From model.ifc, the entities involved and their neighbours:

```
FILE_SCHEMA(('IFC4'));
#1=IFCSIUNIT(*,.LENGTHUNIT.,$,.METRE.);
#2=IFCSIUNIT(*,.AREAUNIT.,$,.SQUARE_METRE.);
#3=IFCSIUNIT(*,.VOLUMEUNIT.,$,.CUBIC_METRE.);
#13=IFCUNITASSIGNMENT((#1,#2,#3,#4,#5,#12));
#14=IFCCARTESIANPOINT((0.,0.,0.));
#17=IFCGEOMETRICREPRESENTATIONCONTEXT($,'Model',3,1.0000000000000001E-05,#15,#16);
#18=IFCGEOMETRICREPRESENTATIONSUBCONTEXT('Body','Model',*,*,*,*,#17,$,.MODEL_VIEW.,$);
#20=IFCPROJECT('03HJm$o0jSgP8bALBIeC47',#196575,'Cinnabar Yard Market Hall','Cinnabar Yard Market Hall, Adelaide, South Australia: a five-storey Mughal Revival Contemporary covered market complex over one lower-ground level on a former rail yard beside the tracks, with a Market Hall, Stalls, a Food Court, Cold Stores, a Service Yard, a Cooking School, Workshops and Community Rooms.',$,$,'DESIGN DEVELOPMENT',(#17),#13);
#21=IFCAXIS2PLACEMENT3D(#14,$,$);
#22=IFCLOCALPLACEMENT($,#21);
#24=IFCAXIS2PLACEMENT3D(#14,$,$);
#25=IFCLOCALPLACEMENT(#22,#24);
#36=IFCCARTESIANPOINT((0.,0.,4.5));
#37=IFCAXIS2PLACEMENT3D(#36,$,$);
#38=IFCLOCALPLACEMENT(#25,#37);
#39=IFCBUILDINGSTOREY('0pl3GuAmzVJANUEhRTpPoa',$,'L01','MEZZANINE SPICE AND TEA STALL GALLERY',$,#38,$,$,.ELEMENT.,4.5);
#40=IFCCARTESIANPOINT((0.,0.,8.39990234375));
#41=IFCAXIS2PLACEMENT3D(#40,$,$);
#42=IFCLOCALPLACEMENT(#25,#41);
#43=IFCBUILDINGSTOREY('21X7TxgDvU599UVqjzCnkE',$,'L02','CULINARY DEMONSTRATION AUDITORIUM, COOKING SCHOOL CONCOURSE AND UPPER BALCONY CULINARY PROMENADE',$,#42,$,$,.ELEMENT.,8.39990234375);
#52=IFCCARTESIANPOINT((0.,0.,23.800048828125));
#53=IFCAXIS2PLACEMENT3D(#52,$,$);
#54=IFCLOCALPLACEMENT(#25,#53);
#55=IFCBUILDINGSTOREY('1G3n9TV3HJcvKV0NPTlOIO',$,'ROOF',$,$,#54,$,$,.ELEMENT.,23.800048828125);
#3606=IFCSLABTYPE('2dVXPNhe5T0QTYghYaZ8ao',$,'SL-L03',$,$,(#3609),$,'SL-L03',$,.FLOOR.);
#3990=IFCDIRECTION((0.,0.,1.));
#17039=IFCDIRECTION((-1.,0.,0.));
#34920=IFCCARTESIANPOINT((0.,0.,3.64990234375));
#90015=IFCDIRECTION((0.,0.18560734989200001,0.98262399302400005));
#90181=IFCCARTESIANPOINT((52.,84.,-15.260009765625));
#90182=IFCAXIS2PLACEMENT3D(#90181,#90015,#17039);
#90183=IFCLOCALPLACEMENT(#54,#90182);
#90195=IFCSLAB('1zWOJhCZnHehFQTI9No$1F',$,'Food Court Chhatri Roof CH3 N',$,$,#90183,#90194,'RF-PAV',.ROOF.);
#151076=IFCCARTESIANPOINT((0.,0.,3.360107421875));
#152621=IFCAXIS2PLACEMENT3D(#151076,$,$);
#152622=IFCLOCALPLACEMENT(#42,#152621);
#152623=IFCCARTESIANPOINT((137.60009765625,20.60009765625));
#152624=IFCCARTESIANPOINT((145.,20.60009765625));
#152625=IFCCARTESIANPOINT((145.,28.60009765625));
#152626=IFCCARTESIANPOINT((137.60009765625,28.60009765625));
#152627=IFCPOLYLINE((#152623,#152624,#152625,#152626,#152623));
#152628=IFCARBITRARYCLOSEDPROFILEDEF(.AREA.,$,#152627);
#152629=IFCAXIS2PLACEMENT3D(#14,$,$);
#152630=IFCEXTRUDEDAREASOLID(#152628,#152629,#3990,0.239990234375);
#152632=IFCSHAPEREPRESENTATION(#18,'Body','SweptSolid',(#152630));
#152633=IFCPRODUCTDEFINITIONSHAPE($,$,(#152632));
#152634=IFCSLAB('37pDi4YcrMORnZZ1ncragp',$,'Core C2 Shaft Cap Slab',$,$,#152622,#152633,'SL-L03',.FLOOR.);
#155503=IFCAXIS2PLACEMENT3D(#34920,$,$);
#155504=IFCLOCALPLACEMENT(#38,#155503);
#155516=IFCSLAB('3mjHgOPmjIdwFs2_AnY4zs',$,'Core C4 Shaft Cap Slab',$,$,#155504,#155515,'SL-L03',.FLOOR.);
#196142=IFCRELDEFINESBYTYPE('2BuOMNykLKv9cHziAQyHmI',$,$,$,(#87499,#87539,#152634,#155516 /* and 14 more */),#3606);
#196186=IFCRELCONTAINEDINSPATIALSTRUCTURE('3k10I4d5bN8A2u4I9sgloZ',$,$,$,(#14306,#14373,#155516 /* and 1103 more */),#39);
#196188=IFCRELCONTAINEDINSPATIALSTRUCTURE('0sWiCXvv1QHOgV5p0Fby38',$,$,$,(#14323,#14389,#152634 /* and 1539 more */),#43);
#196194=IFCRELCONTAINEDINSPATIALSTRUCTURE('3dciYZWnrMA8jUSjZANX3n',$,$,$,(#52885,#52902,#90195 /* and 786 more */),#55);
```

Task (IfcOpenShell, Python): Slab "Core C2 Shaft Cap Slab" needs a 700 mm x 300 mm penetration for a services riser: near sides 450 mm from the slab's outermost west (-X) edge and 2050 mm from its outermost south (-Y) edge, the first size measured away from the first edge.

```python
import numpy as np
import ifcopenshell
import ifcopenshell.api.feature
import ifcopenshell.api.geometry
import ifcopenshell.api.root
import ifcopenshell.geom
import ifcopenshell.util.placement
import ifcopenshell.util.representation
import ifcopenshell.util.shape
import ifcopenshell.util.unit

model = ifcopenshell.open("model.ifc")
unit_scale = ifcopenshell.util.unit.calculate_unit_scale(model)
settings = ifcopenshell.geom.settings()


def volume(element):
    """Net volume in cubic metres, openings subtracted."""
    shape = ifcopenshell.geom.create_shape(settings, element)
    return ifcopenshell.util.shape.get_volume(shape.geometry)


slab = model.by_guid("37pDi4YcrMORnZZ1ncragp")
before = volume(slab)

# Extent in the slab's own axes, in metres. The edges named are its -X and -Y sides.
slab_shape = ifcopenshell.geom.create_shape(settings, slab)
vertices = ifcopenshell.util.shape.get_vertices(slab_shape.geometry)
x_min, y_min, bottom = vertices.min(axis=0)
top = vertices[:, 2].max()

opening = ifcopenshell.api.root.create_entity(model, ifc_class="IfcOpeningElement", name="Services riser opening", predefined_type="OPENING")
context = ifcopenshell.util.representation.get_context(model, "Model", "Body", "MODEL_VIEW")
width, depth = 0.7, 0.3
outline = [(0.0, 0.0), (width, 0.0), (width, depth), (0.0, depth), (0.0, 0.0)]
# Overshoot both faces by 50 mm so the cut is clean.
shape = ifcopenshell.api.geometry.add_slab_representation(
    model, context=context, depth=top - bottom + 0.1, polyline=outline
)
ifcopenshell.api.geometry.assign_representation(model, product=opening, representation=shape)

matrix = ifcopenshell.util.placement.get_local_placement(slab.ObjectPlacement)
matrix[:, 3] = matrix @ np.append(np.array([x_min + 0.45, y_min + 2.05, bottom - 0.05]) / unit_scale, 1.0)
ifcopenshell.api.geometry.edit_object_placement(model, product=opening, matrix=matrix, is_si=False)
ifcopenshell.api.feature.add_feature(model, feature=opening, element=slab)

after = volume(slab)

print(f"slab volume {before:.3f} -> {after:.3f} m3")

model.write("model_edited.ifc")
```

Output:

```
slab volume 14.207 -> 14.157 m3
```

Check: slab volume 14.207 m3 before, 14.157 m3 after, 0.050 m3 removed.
